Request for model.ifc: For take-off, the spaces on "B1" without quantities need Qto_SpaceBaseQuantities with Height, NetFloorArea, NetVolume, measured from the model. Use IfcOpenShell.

First a look at what the model holds.

```python
import ifcopenshell
import ifcopenshell.util.element
import ifcopenshell.util.unit

model = ifcopenshell.open("model.ifc")
print(model.schema)
for unit_type in ("LENGTHUNIT", "AREAUNIT", "VOLUMEUNIT"):
    print(unit_type, ifcopenshell.util.unit.calculate_unit_scale(model, unit_type))
storey = next(s for s in model.by_type("IfcBuildingStorey") if s.Name == "B1")
spaces = [e for e in ifcopenshell.util.element.get_decomposition(storey) if e.is_a("IfcSpace")]
for e in sorted(spaces, key=lambda e: e.id()):
    print(e.id(), e.is_a(), e.Name, list(ifcopenshell.util.element.get_psets(e, qtos_only=True)), sep=" | ")
```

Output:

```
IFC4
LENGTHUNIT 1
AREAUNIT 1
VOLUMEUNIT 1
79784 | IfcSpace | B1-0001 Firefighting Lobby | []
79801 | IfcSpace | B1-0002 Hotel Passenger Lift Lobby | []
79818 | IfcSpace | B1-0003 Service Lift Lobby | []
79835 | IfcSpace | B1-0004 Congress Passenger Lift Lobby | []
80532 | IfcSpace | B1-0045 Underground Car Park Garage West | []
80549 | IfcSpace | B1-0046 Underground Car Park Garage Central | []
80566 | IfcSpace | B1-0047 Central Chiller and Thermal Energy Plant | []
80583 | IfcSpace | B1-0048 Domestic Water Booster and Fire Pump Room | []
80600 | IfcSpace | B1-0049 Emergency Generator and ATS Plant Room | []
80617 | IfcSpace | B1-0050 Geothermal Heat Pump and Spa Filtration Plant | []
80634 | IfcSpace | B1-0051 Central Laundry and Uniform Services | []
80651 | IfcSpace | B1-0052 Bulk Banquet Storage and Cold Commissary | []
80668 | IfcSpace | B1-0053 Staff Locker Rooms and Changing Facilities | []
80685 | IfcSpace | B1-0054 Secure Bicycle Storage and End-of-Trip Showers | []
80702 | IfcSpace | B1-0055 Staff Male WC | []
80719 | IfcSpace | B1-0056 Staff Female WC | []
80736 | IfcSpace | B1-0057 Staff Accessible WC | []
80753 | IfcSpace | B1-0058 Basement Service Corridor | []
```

```python
import ifcopenshell
import ifcopenshell.api.pset
import ifcopenshell.geom
import ifcopenshell.util.element
import ifcopenshell.util.shape
import ifcopenshell.util.unit

model = ifcopenshell.open("model.ifc")
unit_scale = ifcopenshell.util.unit.calculate_unit_scale(model)
area_scale = ifcopenshell.util.unit.calculate_unit_scale(model, "AREAUNIT")
volume_scale = ifcopenshell.util.unit.calculate_unit_scale(model, "VOLUMEUNIT")
settings = ifcopenshell.geom.settings()

storey = next(s for s in model.by_type("IfcBuildingStorey") if s.Name == "B1")
spaces = [e for e in ifcopenshell.util.element.get_decomposition(storey) if e.is_a("IfcSpace")]

for e in sorted(spaces, key=lambda e: e.id()):
    if ifcopenshell.util.element.get_psets(e, qtos_only=True, should_inherit=False):
        continue
    # Geometry comes back in metres, in the element's own axes.
    shape = ifcopenshell.geom.create_shape(settings, e)
    values = {
        "Height": ifcopenshell.util.shape.get_z(shape.geometry) / unit_scale,
        "NetFloorArea": ifcopenshell.util.shape.get_footprint_area(shape.geometry) / area_scale,
        "NetVolume": ifcopenshell.util.shape.get_volume(shape.geometry) / volume_scale,
    }
    qto = ifcopenshell.api.pset.add_qto(model, product=e, name="Qto_SpaceBaseQuantities")
    ifcopenshell.api.pset.edit_qto(model, qto=qto, properties=values)
    print(e.id(), {k: round(v, 3) for k, v in values.items()})

model.write("model_updated.ifc")
```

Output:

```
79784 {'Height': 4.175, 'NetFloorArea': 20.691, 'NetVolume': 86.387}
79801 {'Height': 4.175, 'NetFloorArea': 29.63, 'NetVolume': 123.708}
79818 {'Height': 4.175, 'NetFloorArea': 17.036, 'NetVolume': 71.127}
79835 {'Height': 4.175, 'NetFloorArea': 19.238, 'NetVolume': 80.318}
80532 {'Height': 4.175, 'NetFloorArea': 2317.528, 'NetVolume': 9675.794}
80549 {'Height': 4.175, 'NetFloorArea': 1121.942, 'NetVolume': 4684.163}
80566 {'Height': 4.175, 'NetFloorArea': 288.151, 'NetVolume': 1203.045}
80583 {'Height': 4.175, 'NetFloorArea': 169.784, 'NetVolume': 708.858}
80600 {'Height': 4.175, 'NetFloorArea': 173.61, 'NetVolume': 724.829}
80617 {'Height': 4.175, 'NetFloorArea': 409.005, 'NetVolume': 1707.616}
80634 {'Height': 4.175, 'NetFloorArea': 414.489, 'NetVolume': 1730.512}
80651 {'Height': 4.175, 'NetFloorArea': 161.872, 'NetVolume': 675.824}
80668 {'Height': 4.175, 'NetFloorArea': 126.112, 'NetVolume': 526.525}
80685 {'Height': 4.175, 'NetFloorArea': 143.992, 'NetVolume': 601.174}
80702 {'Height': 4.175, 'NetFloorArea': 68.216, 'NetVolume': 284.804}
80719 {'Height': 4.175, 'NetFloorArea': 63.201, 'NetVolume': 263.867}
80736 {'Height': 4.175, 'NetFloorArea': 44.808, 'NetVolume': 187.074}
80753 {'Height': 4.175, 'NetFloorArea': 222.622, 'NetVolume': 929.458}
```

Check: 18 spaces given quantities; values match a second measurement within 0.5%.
